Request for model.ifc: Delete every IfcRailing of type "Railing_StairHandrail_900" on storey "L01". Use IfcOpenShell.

First a look at what the model holds.

```python
import ifcopenshell
import ifcopenshell.util.element

model = ifcopenshell.open("model.ifc")
print(model.schema)
storey = next(s for s in model.by_type("IfcBuildingStorey") if s.Name == "L01")
railings = [e for e in ifcopenshell.util.element.get_decomposition(storey) if e.is_a("IfcRailing")]
seen = {}
for e in railings:
    element_type = ifcopenshell.util.element.get_type(e)
    name = element_type.Name if element_type not in (None, e) else None
    seen[name] = seen.get(name, 0) + 1
for name, count in sorted(seen.items(), key=str):
    print(count, "x", name)
```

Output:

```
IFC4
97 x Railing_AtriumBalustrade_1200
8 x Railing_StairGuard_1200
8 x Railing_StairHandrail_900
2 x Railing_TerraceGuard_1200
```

```python
import ifcopenshell
import ifcopenshell.api.root
import ifcopenshell.util.element

model = ifcopenshell.open("model.ifc")

storey = next(s for s in model.by_type("IfcBuildingStorey") if s.Name == "L01")
railings = [e for e in ifcopenshell.util.element.get_decomposition(storey) if e.is_a("IfcRailing")]
targets = [e for e in railings if (t := ifcopenshell.util.element.get_type(e)) not in (None, e) and t.Name == "Railing_StairHandrail_900"]

for e in targets:
    ifcopenshell.api.root.remove_product(model, product=e)
print(len(targets), "removed")

model.write("model_updated.ifc")
```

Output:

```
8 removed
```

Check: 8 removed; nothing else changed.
